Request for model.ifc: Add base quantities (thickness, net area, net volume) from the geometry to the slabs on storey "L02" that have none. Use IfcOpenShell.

First a look at what the model holds.

```python
import ifcopenshell
import ifcopenshell.util.element
import ifcopenshell.util.unit

model = ifcopenshell.open("model.ifc")
print(model.schema)
for unit_type in ("LENGTHUNIT", "AREAUNIT", "VOLUMEUNIT"):
    print(unit_type, ifcopenshell.util.unit.calculate_unit_scale(model, unit_type))
storey = next(s for s in model.by_type("IfcBuildingStorey") if s.Name == "L02")
slabs = [e for e in ifcopenshell.util.element.get_decomposition(storey) if e.is_a("IfcSlab")]
for e in sorted(slabs, key=lambda e: e.id()):
    print(e.id(), e.is_a(), e.Name, list(ifcopenshell.util.element.get_psets(e, qtos_only=True)), sep=" | ")
```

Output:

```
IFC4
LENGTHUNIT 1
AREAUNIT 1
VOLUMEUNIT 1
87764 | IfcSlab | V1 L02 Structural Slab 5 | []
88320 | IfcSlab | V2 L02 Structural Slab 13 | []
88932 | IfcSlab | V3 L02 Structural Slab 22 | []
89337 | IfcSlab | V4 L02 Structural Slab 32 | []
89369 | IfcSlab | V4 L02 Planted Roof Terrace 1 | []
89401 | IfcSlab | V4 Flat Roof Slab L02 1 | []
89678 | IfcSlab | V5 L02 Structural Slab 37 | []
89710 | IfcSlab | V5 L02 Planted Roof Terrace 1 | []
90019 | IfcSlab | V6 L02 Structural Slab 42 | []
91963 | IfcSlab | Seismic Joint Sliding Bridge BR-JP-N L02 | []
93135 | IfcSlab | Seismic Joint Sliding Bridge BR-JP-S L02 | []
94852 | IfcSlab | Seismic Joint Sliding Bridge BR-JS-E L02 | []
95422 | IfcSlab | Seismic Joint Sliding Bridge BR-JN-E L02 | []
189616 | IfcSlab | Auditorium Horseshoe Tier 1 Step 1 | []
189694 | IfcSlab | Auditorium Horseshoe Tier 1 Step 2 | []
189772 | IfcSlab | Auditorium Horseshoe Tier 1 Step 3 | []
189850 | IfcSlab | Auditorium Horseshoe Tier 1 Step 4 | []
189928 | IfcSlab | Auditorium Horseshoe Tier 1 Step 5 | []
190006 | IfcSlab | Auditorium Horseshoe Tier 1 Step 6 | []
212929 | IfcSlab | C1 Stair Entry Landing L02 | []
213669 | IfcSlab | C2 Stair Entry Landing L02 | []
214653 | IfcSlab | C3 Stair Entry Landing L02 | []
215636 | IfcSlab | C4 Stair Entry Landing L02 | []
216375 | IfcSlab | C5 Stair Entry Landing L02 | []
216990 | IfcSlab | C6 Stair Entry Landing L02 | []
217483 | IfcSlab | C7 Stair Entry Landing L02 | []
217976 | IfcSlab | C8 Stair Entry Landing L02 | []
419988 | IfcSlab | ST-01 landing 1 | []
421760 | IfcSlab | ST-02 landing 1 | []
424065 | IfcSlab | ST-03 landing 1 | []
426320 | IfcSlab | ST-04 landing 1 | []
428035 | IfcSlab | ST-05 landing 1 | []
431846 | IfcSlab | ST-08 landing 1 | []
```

```python
import ifcopenshell
import ifcopenshell.api.pset
import ifcopenshell.geom
import ifcopenshell.util.element
import ifcopenshell.util.shape
import ifcopenshell.util.unit

model = ifcopenshell.open("model.ifc")
unit_scale = ifcopenshell.util.unit.calculate_unit_scale(model)
area_scale = ifcopenshell.util.unit.calculate_unit_scale(model, "AREAUNIT")
volume_scale = ifcopenshell.util.unit.calculate_unit_scale(model, "VOLUMEUNIT")
settings = ifcopenshell.geom.settings()

storey = next(s for s in model.by_type("IfcBuildingStorey") if s.Name == "L02")
slabs = [e for e in ifcopenshell.util.element.get_decomposition(storey) if e.is_a("IfcSlab")]

for e in sorted(slabs, key=lambda e: e.id()):
    if ifcopenshell.util.element.get_psets(e, qtos_only=True, should_inherit=False):
        continue
    # Geometry comes back in metres, in the element's own axes.
    shape = ifcopenshell.geom.create_shape(settings, e)
    values = {
        "Width": ifcopenshell.util.shape.get_z(shape.geometry) / unit_scale,
        "NetArea": ifcopenshell.util.shape.get_footprint_area(shape.geometry) / area_scale,
        "NetVolume": ifcopenshell.util.shape.get_volume(shape.geometry) / volume_scale,
    }
    qto = ifcopenshell.api.pset.add_qto(model, product=e, name="Qto_SlabBaseQuantities")
    ifcopenshell.api.pset.edit_qto(model, qto=qto, properties=values)
    print(e.id(), {k: round(v, 3) for k, v in values.items()})

model.write("model-out.ifc")
```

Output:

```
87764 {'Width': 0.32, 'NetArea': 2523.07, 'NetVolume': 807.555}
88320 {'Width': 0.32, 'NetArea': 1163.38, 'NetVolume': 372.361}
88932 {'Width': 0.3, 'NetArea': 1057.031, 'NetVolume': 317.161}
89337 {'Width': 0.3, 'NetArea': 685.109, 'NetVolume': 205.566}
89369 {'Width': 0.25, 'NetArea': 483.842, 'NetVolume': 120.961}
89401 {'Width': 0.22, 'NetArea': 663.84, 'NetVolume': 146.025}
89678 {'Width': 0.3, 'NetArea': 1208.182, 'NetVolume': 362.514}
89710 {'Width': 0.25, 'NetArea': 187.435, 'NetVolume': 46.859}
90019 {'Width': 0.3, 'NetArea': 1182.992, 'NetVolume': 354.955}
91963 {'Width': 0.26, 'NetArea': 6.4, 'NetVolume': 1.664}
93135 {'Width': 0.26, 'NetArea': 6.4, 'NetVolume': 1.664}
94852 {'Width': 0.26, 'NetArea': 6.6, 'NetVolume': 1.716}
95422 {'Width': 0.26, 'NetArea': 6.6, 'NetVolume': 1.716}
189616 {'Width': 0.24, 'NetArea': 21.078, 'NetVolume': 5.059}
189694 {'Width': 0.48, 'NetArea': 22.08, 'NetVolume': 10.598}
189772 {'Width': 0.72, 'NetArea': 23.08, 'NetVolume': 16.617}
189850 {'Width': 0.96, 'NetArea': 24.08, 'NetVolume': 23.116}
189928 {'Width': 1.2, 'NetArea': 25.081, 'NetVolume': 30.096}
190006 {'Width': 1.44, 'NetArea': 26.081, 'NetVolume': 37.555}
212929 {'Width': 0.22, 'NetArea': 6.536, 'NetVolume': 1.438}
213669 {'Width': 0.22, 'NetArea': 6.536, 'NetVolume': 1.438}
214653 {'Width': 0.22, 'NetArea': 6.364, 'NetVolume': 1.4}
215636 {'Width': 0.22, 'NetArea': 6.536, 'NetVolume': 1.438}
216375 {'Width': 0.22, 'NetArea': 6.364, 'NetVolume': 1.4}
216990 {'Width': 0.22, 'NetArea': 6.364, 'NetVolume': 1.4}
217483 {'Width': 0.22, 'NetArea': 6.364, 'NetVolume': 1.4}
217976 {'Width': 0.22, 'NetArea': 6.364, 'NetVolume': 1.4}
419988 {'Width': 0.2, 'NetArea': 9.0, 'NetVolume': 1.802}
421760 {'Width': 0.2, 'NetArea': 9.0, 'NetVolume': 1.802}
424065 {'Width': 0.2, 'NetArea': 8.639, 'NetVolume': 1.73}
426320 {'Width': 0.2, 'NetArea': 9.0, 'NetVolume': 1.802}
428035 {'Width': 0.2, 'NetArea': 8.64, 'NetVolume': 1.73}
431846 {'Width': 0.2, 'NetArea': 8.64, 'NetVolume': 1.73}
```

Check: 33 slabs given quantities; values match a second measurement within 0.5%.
